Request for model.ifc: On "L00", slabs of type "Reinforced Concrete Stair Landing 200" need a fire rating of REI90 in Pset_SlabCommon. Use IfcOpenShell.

First a look at what the model holds.

```python
import ifcopenshell
import ifcopenshell.util.element

model = ifcopenshell.open("model.ifc")
print(model.schema)
storey = next(s for s in model.by_type("IfcBuildingStorey") if s.Name == "L00")
slabs = [e for e in ifcopenshell.util.element.get_decomposition(storey) if e.is_a("IfcSlab")]
seen = {}
for e in slabs:
    element_type = ifcopenshell.util.element.get_type(e)
    key = (element_type.Name if element_type != e and element_type else None, ifcopenshell.util.element.get_pset(e, "Pset_SlabCommon", "FireRating"))
    seen[key] = seen.get(key, 0) + 1
for (name, value), count in sorted(seen.items(), key=str):
    print(count, "x", name, "|", value)
```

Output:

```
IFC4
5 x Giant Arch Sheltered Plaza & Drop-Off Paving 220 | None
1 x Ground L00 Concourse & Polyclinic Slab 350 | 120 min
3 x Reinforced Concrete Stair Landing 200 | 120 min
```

```python
import ifcopenshell
import ifcopenshell.api.pset
import ifcopenshell.util.element

model = ifcopenshell.open("model.ifc")

storey = next(s for s in model.by_type("IfcBuildingStorey") if s.Name == "L00")
slabs = [e for e in ifcopenshell.util.element.get_decomposition(storey) if e.is_a("IfcSlab")]

count = 0
for e in slabs:
    element_type = ifcopenshell.util.element.get_type(e)
    if element_type in (None, e) or element_type.Name != "Reinforced Concrete Stair Landing 200":
        continue
    # add_pset returns the element's existing set when there is one.
    pset = ifcopenshell.api.pset.add_pset(model, product=e, name="Pset_SlabCommon")
    ifcopenshell.api.pset.edit_pset(model, pset=pset, properties={"FireRating": "REI90"})
    count += 1

print(count, "slabs updated")

model.write("model_edited.ifc")
```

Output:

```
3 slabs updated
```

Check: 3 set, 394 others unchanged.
